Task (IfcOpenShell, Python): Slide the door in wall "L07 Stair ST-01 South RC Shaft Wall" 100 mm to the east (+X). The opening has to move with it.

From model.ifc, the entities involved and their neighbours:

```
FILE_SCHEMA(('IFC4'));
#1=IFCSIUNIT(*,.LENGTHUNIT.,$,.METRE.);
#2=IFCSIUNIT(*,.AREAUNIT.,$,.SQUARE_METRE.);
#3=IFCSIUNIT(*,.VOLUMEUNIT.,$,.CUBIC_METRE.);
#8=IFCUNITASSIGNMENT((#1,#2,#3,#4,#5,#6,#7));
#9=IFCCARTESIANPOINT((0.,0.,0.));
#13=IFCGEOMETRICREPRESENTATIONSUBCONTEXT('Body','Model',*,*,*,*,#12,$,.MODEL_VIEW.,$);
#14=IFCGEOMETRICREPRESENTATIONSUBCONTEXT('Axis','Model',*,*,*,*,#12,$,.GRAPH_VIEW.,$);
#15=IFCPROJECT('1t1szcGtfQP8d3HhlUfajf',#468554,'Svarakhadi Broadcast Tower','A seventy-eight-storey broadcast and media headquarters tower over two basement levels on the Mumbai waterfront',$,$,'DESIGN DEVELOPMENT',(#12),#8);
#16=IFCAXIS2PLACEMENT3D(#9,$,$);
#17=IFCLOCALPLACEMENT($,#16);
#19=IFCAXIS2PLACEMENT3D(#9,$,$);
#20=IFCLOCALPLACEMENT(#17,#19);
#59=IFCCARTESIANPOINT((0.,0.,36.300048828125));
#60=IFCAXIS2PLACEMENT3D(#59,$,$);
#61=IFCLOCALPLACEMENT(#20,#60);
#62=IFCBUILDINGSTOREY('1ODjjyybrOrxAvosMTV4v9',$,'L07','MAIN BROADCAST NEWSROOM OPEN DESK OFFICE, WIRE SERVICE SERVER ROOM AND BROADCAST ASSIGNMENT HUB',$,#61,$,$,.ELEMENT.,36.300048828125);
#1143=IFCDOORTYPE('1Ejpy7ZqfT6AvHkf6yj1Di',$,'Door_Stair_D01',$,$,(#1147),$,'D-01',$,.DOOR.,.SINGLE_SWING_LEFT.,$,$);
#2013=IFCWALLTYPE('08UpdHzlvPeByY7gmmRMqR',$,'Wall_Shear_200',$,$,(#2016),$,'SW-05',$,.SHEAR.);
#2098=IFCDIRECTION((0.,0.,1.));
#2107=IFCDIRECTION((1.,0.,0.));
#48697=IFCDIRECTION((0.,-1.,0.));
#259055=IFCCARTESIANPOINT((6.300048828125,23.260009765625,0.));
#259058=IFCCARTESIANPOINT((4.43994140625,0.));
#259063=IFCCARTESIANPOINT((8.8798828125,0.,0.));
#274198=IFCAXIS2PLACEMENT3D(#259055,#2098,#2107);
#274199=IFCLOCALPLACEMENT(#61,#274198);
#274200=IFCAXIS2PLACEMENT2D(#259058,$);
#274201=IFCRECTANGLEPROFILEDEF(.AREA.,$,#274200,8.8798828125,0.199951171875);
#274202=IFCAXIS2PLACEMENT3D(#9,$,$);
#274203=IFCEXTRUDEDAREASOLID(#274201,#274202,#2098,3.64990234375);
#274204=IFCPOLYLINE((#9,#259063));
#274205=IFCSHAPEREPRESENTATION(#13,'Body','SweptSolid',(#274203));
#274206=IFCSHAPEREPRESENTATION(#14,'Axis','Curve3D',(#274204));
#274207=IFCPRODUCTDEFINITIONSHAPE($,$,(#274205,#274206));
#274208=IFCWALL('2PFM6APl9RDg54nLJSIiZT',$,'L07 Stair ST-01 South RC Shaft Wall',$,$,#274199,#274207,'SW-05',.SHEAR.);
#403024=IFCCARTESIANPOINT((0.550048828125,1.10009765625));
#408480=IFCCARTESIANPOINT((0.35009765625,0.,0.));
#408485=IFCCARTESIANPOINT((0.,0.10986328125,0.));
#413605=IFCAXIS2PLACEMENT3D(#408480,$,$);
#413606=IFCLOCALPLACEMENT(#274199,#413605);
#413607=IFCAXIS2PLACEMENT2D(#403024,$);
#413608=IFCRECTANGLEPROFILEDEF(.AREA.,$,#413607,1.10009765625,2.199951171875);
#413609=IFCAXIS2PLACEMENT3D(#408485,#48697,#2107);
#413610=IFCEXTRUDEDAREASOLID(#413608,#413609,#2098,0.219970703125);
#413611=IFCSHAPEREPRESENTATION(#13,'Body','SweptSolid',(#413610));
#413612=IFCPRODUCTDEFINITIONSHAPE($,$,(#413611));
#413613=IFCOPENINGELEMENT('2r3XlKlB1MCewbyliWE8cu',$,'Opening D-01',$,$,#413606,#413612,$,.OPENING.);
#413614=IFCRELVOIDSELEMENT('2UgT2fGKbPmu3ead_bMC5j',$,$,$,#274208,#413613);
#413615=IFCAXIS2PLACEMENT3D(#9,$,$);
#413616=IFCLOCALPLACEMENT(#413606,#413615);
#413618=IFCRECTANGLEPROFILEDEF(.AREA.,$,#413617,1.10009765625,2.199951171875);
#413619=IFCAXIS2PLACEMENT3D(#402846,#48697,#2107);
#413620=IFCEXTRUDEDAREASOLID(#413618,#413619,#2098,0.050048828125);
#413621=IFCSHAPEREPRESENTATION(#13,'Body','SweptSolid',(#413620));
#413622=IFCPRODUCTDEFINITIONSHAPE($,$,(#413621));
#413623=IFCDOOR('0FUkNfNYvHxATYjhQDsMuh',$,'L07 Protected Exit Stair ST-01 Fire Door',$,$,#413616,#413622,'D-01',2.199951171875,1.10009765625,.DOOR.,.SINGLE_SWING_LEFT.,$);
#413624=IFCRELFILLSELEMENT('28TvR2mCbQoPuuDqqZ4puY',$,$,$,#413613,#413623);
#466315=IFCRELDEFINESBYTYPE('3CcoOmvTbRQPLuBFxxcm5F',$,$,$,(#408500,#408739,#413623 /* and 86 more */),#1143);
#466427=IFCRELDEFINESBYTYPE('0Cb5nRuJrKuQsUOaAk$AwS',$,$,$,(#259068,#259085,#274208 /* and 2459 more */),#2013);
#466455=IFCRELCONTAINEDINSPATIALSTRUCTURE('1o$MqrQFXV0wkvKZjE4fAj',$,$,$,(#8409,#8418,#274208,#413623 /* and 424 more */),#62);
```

```python
import ifcopenshell
import ifcopenshell.api.geometry
import ifcopenshell.util.placement
import ifcopenshell.util.unit

model = ifcopenshell.open("model.ifc")
unit_scale = ifcopenshell.util.unit.calculate_unit_scale(model)

door = model.by_guid("0FUkNfNYvHxATYjhQDsMuh")
opening = door.FillsVoids[0].RelatingOpeningElement
wall = opening.VoidsElements[0].RelatingBuildingElement

wall_matrix = ifcopenshell.util.placement.get_local_placement(wall.ObjectPlacement)
shift = wall_matrix[:3, 0] * 0.1 / unit_scale
before = ifcopenshell.util.placement.get_local_placement(door.ObjectPlacement)[:3, 3].copy()

# The door is placed relative to its opening, so it follows when the opening moves.
matrix = ifcopenshell.util.placement.get_local_placement(opening.ObjectPlacement)
matrix[:3, 3] += shift
ifcopenshell.api.geometry.edit_object_placement(
    model, product=opening, matrix=matrix, is_si=False, should_transform_children=True
)

after = ifcopenshell.util.placement.get_local_placement(door.ObjectPlacement)[:3, 3]
print("door moved by", (after - before).round(3) + 0.0)

model.write("model-out.ifc")
```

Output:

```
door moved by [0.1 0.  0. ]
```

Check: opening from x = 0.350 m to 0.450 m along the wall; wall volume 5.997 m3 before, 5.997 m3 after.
